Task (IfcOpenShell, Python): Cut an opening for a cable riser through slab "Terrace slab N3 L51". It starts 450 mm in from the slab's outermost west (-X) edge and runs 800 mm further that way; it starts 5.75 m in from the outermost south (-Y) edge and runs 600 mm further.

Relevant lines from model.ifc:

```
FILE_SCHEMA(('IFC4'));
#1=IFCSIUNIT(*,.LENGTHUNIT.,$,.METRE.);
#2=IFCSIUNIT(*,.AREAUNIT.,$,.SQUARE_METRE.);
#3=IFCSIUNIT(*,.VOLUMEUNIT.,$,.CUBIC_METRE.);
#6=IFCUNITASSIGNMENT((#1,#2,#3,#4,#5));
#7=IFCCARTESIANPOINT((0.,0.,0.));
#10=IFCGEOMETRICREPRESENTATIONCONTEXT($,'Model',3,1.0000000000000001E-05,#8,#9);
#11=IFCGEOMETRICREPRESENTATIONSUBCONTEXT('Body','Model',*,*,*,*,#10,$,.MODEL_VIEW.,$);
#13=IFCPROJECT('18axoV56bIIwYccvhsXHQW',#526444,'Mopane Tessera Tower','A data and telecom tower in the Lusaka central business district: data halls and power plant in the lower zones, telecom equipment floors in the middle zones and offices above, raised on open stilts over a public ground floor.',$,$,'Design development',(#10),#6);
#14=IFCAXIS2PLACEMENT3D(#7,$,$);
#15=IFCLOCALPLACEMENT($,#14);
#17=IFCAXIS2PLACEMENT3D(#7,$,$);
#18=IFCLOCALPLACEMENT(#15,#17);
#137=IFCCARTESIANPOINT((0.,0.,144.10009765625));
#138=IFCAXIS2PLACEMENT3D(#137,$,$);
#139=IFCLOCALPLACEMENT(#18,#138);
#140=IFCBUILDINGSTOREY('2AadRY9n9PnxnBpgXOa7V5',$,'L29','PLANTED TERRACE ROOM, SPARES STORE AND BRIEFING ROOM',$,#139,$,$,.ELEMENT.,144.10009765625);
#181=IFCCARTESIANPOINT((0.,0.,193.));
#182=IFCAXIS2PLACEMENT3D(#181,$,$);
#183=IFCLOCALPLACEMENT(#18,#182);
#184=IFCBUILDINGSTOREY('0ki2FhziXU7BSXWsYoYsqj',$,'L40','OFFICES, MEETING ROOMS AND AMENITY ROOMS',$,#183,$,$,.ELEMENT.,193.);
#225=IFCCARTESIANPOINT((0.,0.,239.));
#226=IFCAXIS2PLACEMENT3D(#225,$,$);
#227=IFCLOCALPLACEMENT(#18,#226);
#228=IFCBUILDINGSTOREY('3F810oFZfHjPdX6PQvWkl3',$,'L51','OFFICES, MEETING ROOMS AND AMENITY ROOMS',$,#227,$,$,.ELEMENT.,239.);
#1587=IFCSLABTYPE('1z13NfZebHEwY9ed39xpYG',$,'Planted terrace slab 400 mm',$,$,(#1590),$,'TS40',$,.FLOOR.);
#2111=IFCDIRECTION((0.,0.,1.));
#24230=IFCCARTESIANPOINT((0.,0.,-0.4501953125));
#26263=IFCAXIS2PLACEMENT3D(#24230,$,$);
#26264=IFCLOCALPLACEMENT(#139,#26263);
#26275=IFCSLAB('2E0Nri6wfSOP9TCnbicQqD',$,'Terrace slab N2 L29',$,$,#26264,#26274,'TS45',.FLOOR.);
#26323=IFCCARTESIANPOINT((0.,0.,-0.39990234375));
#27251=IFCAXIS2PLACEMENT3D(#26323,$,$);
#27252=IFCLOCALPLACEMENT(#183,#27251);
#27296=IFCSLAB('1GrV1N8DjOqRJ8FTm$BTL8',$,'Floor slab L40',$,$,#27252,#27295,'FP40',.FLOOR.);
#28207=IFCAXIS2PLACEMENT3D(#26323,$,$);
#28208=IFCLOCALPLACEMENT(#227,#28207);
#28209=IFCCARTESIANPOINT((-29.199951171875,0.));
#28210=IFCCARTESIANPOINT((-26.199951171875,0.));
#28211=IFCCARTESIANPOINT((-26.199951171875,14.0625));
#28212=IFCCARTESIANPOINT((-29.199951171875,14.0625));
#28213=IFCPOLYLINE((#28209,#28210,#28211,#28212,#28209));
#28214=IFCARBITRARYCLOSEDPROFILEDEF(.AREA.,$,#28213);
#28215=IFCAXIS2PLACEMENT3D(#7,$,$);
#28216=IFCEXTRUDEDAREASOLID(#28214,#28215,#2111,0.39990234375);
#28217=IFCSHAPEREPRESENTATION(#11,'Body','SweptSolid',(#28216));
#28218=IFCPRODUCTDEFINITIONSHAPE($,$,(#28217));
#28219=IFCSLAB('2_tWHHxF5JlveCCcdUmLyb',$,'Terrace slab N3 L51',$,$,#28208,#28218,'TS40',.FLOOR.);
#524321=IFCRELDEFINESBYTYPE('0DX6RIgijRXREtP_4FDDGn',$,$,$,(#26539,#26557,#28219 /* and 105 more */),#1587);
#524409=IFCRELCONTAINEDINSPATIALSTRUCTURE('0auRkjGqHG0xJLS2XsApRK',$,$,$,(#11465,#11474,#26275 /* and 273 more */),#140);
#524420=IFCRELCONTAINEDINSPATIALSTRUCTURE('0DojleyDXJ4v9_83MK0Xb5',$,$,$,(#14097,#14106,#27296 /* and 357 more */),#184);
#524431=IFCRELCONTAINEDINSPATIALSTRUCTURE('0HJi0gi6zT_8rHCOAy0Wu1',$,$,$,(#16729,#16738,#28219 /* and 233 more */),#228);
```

```python
import numpy as np
import ifcopenshell
import ifcopenshell.api.feature
import ifcopenshell.api.geometry
import ifcopenshell.api.root
import ifcopenshell.geom
import ifcopenshell.util.placement
import ifcopenshell.util.representation
import ifcopenshell.util.shape
import ifcopenshell.util.unit

model = ifcopenshell.open("model.ifc")
unit_scale = ifcopenshell.util.unit.calculate_unit_scale(model)
settings = ifcopenshell.geom.settings()


def volume(element):
    """Net volume in cubic metres, openings subtracted."""
    shape = ifcopenshell.geom.create_shape(settings, element)
    return ifcopenshell.util.shape.get_volume(shape.geometry)


slab = model.by_guid("2_tWHHxF5JlveCCcdUmLyb")
before = volume(slab)

# Extent in the slab's own axes, in metres. The edges named are its -X and -Y sides.
slab_shape = ifcopenshell.geom.create_shape(settings, slab)
vertices = ifcopenshell.util.shape.get_vertices(slab_shape.geometry)
x_min, y_min, bottom = vertices.min(axis=0)
top = vertices[:, 2].max()

opening = ifcopenshell.api.root.create_entity(model, ifc_class="IfcOpeningElement", name="Cable riser opening", predefined_type="OPENING")
context = ifcopenshell.util.representation.get_context(model, "Model", "Body", "MODEL_VIEW")
width, depth = 0.8, 0.6
outline = [(0.0, 0.0), (width, 0.0), (width, depth), (0.0, depth), (0.0, 0.0)]
# Overshoot both faces by 50 mm so the cut is clean.
shape = ifcopenshell.api.geometry.add_slab_representation(
    model, context=context, depth=top - bottom + 0.1, polyline=outline
)
ifcopenshell.api.geometry.assign_representation(model, product=opening, representation=shape)

matrix = ifcopenshell.util.placement.get_local_placement(slab.ObjectPlacement)
matrix[:, 3] = matrix @ np.append(np.array([x_min + 0.45, y_min + 5.75, bottom - 0.05]) / unit_scale, 1.0)
ifcopenshell.api.geometry.edit_object_placement(model, product=opening, matrix=matrix, is_si=False)
ifcopenshell.api.feature.add_feature(model, feature=opening, element=slab)

after = volume(slab)

print(f"slab volume {before:.3f} -> {after:.3f} m3")

model.write("model_v2.ifc")
```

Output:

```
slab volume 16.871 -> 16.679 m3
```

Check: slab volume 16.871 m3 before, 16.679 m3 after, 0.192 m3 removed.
